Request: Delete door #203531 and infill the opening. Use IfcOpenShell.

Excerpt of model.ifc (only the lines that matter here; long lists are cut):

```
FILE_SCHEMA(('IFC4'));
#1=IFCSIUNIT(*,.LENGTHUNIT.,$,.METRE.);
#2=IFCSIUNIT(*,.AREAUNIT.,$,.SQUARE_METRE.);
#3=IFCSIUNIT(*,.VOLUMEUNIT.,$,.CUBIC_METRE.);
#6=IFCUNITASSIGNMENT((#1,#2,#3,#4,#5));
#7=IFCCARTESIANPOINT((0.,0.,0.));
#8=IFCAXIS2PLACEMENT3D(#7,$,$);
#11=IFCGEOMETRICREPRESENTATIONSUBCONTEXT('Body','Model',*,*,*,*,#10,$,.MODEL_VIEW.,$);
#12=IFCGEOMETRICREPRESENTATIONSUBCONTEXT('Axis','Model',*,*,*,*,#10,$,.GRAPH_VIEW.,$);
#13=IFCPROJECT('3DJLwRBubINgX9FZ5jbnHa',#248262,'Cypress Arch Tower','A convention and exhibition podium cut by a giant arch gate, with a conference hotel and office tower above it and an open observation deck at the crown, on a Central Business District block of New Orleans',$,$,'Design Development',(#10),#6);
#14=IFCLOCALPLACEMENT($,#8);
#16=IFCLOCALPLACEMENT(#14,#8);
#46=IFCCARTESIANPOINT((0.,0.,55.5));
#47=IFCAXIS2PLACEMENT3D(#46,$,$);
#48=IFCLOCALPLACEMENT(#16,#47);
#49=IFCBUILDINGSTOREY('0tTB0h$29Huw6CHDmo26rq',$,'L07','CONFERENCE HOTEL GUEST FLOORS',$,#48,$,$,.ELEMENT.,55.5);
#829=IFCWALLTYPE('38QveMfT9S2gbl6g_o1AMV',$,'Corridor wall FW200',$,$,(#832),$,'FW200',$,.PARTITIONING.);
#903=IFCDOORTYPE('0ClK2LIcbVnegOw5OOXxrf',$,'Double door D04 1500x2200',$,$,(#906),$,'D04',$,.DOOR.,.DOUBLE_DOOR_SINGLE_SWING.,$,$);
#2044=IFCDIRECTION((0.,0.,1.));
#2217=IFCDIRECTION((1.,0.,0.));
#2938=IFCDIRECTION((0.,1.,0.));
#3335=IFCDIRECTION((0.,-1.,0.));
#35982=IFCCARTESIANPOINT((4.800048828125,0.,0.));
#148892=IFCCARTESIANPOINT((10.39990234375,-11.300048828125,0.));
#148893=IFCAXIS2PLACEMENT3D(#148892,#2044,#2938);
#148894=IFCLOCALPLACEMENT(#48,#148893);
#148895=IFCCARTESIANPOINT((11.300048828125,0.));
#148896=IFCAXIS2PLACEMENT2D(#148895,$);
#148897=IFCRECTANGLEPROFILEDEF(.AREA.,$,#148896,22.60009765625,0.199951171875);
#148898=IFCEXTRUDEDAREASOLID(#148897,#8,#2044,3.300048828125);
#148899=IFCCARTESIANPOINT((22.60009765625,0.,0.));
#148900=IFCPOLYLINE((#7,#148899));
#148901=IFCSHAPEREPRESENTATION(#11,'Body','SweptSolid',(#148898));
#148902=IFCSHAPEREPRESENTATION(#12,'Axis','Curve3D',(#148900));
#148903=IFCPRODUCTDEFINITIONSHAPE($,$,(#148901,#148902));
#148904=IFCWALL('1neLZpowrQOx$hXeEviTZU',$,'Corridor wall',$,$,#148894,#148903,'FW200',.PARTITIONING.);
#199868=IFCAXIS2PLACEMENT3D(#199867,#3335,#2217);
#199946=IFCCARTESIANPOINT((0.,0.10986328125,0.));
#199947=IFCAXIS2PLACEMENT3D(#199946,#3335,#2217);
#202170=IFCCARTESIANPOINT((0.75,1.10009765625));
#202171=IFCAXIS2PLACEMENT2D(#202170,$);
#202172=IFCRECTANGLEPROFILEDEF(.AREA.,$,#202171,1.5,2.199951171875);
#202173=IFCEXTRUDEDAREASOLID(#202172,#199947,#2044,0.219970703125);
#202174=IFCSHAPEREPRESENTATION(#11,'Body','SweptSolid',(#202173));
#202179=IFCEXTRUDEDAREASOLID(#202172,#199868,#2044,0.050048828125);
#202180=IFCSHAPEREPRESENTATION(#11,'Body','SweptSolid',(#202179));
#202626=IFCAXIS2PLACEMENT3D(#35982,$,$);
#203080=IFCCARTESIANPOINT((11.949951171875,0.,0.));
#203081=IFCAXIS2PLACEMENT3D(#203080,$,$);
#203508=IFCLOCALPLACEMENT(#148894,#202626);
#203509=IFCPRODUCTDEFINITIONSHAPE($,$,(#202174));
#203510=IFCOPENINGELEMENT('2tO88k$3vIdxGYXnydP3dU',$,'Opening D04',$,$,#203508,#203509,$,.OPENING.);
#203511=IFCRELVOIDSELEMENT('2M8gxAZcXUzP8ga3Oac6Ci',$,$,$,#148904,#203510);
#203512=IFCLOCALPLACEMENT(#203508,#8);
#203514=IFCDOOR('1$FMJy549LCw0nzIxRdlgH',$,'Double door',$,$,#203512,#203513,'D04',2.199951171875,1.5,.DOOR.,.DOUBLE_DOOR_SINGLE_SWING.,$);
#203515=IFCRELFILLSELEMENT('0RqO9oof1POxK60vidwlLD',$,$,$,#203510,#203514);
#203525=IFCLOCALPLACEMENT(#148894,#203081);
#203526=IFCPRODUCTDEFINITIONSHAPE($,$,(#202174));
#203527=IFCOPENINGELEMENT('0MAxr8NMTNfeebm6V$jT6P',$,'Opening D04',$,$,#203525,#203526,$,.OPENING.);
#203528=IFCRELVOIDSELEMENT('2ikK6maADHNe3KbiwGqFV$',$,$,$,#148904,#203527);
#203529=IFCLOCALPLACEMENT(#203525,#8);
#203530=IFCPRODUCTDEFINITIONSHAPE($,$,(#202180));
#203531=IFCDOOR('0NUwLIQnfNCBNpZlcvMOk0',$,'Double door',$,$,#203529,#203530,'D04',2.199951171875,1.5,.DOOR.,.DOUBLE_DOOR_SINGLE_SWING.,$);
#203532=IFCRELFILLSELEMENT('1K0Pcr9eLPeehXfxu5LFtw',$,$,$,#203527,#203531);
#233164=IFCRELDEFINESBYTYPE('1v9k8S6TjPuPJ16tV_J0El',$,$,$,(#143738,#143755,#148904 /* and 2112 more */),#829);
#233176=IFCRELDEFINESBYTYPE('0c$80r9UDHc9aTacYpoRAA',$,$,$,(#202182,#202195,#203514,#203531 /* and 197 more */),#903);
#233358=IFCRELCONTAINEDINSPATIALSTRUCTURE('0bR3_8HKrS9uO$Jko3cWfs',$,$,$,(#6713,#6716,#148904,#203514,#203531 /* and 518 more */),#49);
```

```python
import ifcopenshell
import ifcopenshell.api.feature
import ifcopenshell.api.root
import ifcopenshell.geom
import ifcopenshell.util.shape

model = ifcopenshell.open("model.ifc")
settings = ifcopenshell.geom.settings()


def volume(element):
    """Net volume in cubic metres, openings subtracted."""
    shape = ifcopenshell.geom.create_shape(settings, element)
    return ifcopenshell.util.shape.get_volume(shape.geometry)


door = model.by_guid("0NUwLIQnfNCBNpZlcvMOk0")
opening = door.FillsVoids[0].RelatingOpeningElement
wall = opening.VoidsElements[0].RelatingBuildingElement
before = volume(wall)

ifcopenshell.api.root.remove_product(model, product=door)
ifcopenshell.api.feature.remove_feature(model, feature=opening)

after = volume(wall)

print(f"wall volume {before:.3f} -> {after:.3f} m3")

model.write("model_rev.ifc")
```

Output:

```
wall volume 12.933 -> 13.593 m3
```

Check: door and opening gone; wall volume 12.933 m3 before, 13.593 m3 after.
